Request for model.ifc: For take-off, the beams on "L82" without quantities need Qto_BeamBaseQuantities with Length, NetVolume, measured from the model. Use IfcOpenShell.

First a look at what the model holds.

```python
import ifcopenshell
import ifcopenshell.util.element
import ifcopenshell.util.unit

model = ifcopenshell.open("model.ifc")
print(model.schema)
for unit_type in ("LENGTHUNIT", "AREAUNIT", "VOLUMEUNIT"):
    print(unit_type, ifcopenshell.util.unit.calculate_unit_scale(model, unit_type))
storey = next(s for s in model.by_type("IfcBuildingStorey") if s.Name == "L82")
beams = [e for e in ifcopenshell.util.element.get_decomposition(storey) if e.is_a("IfcBeam")]
for e in sorted(beams, key=lambda e: e.id()):
    print(e.id(), e.is_a(), e.Name, list(ifcopenshell.util.element.get_psets(e, qtos_only=True)), sep=" | ")
```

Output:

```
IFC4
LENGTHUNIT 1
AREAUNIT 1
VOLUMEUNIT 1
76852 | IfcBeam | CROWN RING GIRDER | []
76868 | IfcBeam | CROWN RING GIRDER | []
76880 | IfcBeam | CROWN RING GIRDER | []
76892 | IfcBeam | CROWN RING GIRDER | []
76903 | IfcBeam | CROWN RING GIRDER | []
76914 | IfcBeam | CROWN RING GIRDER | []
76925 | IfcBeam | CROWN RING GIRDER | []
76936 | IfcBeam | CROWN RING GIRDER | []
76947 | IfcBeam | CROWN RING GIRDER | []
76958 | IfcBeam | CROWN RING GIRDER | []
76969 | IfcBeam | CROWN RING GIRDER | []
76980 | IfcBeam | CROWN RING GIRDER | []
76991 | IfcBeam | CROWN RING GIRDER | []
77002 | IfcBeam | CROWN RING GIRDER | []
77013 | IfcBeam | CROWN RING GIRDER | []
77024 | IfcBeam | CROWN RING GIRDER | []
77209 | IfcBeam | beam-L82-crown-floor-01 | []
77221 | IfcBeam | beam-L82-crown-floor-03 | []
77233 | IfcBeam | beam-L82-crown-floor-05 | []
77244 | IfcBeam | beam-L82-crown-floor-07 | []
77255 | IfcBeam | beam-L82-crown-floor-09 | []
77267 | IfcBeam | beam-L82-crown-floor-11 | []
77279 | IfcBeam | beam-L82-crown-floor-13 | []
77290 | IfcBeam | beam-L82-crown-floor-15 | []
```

```python
import ifcopenshell
import ifcopenshell.api.pset
import ifcopenshell.geom
import ifcopenshell.util.element
import ifcopenshell.util.shape
import ifcopenshell.util.unit

model = ifcopenshell.open("model.ifc")
unit_scale = ifcopenshell.util.unit.calculate_unit_scale(model)
volume_scale = ifcopenshell.util.unit.calculate_unit_scale(model, "VOLUMEUNIT")
settings = ifcopenshell.geom.settings()

storey = next(s for s in model.by_type("IfcBuildingStorey") if s.Name == "L82")
beams = [e for e in ifcopenshell.util.element.get_decomposition(storey) if e.is_a("IfcBeam")]

for e in sorted(beams, key=lambda e: e.id()):
    if ifcopenshell.util.element.get_psets(e, qtos_only=True, should_inherit=False):
        continue
    # Geometry comes back in metres, in the element's own axes.
    shape = ifcopenshell.geom.create_shape(settings, e)
    values = {
        "Length": ifcopenshell.util.shape.get_max_xyz(shape.geometry) / unit_scale,
        "NetVolume": ifcopenshell.util.shape.get_volume(shape.geometry) / volume_scale,
    }
    qto = ifcopenshell.api.pset.add_qto(model, product=e, name="Qto_BeamBaseQuantities")
    ifcopenshell.api.pset.edit_qto(model, qto=qto, properties=values)
    print(e.id(), {k: round(v, 3) for k, v in values.items()})

model.write("model_v2.ifc")
```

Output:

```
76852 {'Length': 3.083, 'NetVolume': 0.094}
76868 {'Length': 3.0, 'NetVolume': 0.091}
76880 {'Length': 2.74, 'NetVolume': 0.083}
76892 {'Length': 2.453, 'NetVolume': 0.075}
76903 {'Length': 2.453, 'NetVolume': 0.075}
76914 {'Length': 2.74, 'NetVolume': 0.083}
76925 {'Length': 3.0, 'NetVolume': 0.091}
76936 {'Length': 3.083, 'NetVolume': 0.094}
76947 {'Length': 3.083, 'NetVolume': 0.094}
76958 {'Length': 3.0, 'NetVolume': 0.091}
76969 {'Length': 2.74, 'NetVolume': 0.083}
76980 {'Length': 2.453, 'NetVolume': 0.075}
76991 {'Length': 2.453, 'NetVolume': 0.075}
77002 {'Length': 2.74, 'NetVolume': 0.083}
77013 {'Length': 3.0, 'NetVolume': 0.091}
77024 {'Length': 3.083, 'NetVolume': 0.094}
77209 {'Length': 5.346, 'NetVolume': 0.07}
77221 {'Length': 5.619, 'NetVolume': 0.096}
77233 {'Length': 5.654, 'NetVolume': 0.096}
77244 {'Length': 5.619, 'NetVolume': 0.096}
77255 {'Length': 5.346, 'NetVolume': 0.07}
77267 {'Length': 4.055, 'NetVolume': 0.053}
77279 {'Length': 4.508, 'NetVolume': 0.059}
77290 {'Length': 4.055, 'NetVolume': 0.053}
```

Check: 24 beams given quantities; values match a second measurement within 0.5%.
